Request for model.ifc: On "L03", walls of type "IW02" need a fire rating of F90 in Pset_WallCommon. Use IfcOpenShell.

First a look at what the model holds.

```python
import ifcopenshell
import ifcopenshell.util.element

model = ifcopenshell.open("model.ifc")
print(model.schema)
storey = next(s for s in model.by_type("IfcBuildingStorey") if s.Name == "L03")
walls = [e for e in ifcopenshell.util.element.get_decomposition(storey) if e.is_a("IfcWall")]
seen = {}
for e in walls:
    element_type = ifcopenshell.util.element.get_type(e)
    key = (element_type.Name if element_type != e and element_type else None, ifcopenshell.util.element.get_pset(e, "Pset_WallCommon", "FireRating"))
    seen[key] = seen.get(key, 0) + 1
for (name, value), count in sorted(seen.items(), key=str):
    print(count, "x", name, "|", value)
```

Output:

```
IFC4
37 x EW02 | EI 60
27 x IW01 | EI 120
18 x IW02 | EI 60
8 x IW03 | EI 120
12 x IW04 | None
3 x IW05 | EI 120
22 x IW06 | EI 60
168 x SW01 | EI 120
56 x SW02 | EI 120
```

```python
import ifcopenshell
import ifcopenshell.api.pset
import ifcopenshell.util.element

model = ifcopenshell.open("model.ifc")

storey = next(s for s in model.by_type("IfcBuildingStorey") if s.Name == "L03")
walls = [e for e in ifcopenshell.util.element.get_decomposition(storey) if e.is_a("IfcWall")]

count = 0
for e in walls:
    element_type = ifcopenshell.util.element.get_type(e)
    if element_type in (None, e) or element_type.Name != "IW02":
        continue
    # add_pset returns the element's existing set when there is one.
    pset = ifcopenshell.api.pset.add_pset(model, product=e, name="Pset_WallCommon")
    ifcopenshell.api.pset.edit_pset(model, pset=pset, properties={"FireRating": "F90"})
    count += 1

print(count, "walls updated")

model.write("model-out.ifc")
```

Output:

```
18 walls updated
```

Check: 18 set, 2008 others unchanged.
